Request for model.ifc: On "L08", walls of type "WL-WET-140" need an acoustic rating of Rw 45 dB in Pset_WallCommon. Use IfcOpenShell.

First a look at what the model holds.

```python
import ifcopenshell
import ifcopenshell.util.element

model = ifcopenshell.open("model.ifc")
print(model.schema)
storey = next(s for s in model.by_type("IfcBuildingStorey") if s.Name == "L08")
walls = [e for e in ifcopenshell.util.element.get_decomposition(storey) if e.is_a("IfcWall")]
seen = {}
for e in walls:
    element_type = ifcopenshell.util.element.get_type(e)
    key = (element_type.Name if element_type != e and element_type else None, ifcopenshell.util.element.get_pset(e, "Pset_WallCommon", "AcousticRating"))
    seen[key] = seen.get(key, 0) + 1
for (name, value), count in sorted(seen.items(), key=str):
    print(count, "x", name, "|", value)
```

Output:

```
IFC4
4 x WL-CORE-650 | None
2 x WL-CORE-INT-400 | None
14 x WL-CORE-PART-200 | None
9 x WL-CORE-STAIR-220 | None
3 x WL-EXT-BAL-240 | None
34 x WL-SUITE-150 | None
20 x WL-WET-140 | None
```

```python
import ifcopenshell
import ifcopenshell.api.pset
import ifcopenshell.util.element

model = ifcopenshell.open("model.ifc")

storey = next(s for s in model.by_type("IfcBuildingStorey") if s.Name == "L08")
walls = [e for e in ifcopenshell.util.element.get_decomposition(storey) if e.is_a("IfcWall")]

count = 0
for e in walls:
    element_type = ifcopenshell.util.element.get_type(e)
    if element_type in (None, e) or element_type.Name != "WL-WET-140":
        continue
    # add_pset returns the element's existing set when there is one.
    pset = ifcopenshell.api.pset.add_pset(model, product=e, name="Pset_WallCommon")
    ifcopenshell.api.pset.edit_pset(model, pset=pset, properties={"AcousticRating": "Rw 45 dB"})
    count += 1

print(count, "walls updated")

model.write("model_updated.ifc")
```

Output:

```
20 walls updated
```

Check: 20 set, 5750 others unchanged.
